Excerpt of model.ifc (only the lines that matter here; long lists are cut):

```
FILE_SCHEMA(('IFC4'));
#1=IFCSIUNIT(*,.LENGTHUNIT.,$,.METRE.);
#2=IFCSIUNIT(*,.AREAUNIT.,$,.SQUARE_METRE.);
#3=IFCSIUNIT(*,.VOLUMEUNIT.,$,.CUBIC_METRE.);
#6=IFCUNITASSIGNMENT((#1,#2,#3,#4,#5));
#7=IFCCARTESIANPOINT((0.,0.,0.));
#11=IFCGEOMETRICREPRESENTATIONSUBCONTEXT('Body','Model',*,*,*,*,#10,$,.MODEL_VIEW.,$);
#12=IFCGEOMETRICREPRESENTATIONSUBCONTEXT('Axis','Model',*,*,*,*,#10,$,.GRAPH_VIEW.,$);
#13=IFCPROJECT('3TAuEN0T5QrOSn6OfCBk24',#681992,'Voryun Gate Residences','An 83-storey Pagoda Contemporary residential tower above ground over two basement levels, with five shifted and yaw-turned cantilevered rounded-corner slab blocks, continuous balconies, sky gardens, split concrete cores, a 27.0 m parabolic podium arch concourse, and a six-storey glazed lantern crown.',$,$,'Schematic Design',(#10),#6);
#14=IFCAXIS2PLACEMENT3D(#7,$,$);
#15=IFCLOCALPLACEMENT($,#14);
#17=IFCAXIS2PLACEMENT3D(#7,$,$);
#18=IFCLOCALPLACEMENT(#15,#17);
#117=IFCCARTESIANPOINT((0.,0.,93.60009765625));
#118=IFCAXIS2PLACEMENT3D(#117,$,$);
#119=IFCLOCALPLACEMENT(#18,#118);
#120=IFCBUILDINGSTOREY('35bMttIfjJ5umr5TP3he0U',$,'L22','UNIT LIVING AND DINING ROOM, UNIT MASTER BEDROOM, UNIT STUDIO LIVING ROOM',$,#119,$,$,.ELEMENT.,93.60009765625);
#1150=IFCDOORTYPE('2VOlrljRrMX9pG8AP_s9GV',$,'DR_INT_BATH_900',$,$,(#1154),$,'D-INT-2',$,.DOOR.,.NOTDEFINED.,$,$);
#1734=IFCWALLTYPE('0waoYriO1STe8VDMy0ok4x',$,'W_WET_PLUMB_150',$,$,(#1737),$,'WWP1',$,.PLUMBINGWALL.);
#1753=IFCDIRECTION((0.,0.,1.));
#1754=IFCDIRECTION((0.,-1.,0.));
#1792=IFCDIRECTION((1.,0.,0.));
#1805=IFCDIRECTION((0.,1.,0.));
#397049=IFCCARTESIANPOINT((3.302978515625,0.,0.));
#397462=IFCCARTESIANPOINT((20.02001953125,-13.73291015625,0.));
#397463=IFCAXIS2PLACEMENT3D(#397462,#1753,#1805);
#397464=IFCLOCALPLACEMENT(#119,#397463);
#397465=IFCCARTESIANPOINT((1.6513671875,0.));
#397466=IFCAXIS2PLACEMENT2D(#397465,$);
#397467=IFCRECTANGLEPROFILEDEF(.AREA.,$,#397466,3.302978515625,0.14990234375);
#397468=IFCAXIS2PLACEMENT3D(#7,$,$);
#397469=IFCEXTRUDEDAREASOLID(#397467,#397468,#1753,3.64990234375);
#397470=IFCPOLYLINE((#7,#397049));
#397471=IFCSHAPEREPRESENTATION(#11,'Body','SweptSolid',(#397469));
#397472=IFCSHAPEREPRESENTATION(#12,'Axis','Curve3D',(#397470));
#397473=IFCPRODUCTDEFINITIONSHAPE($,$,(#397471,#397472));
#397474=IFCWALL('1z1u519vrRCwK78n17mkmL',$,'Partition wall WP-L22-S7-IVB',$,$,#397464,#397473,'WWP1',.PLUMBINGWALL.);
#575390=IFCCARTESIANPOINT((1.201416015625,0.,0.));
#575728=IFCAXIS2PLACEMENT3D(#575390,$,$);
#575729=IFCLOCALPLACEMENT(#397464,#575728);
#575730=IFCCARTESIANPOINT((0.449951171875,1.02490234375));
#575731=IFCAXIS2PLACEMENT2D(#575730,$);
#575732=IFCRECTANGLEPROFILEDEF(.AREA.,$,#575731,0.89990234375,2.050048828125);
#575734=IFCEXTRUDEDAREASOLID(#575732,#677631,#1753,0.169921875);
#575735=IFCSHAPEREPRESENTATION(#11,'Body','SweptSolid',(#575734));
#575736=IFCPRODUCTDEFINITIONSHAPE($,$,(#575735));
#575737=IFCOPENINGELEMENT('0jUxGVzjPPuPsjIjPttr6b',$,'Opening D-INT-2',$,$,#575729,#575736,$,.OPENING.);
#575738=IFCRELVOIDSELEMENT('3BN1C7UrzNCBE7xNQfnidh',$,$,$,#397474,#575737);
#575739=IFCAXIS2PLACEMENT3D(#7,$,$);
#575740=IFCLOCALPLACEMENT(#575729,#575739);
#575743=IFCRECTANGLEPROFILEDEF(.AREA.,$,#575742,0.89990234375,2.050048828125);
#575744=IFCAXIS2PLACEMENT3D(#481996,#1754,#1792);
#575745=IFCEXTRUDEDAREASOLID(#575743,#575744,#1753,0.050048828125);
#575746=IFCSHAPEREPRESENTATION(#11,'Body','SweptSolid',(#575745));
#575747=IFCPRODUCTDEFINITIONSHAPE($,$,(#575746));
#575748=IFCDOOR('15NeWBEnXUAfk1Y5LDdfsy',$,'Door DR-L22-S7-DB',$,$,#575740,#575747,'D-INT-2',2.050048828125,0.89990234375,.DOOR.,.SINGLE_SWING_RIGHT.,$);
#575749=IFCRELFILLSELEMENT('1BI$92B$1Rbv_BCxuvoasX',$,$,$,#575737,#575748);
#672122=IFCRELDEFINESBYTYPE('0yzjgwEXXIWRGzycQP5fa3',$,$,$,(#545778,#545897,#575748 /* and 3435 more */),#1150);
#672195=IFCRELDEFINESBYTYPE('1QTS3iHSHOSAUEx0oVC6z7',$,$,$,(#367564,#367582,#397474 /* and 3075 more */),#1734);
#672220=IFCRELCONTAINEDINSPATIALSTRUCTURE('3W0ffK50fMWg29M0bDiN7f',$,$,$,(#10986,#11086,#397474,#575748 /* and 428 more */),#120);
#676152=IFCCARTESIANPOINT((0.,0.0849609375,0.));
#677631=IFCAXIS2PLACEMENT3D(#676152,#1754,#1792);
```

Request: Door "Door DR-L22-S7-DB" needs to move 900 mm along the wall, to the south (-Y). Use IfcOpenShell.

```python
import ifcopenshell
import ifcopenshell.api.geometry
import ifcopenshell.util.placement

model = ifcopenshell.open("model.ifc")

door = model.by_guid("15NeWBEnXUAfk1Y5LDdfsy")
opening = door.FillsVoids[0].RelatingOpeningElement
wall = opening.VoidsElements[0].RelatingBuildingElement

wall_matrix = ifcopenshell.util.placement.get_local_placement(wall.ObjectPlacement)
shift = wall_matrix[:3, 0] * -0.9
before = ifcopenshell.util.placement.get_local_placement(door.ObjectPlacement)[:3, 3].copy()

# The door is placed relative to its opening, so it follows when the opening moves.
matrix = ifcopenshell.util.placement.get_local_placement(opening.ObjectPlacement)
matrix[:3, 3] += shift
ifcopenshell.api.geometry.edit_object_placement(
    model, product=opening, matrix=matrix, is_si=False, should_transform_children=True
)

after = ifcopenshell.util.placement.get_local_placement(door.ObjectPlacement)[:3, 3]
print("door moved by", (after - before).round(3) + 0.0)

model.write("model-out.ifc")
```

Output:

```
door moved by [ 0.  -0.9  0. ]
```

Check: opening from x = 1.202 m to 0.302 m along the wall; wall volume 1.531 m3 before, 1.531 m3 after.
